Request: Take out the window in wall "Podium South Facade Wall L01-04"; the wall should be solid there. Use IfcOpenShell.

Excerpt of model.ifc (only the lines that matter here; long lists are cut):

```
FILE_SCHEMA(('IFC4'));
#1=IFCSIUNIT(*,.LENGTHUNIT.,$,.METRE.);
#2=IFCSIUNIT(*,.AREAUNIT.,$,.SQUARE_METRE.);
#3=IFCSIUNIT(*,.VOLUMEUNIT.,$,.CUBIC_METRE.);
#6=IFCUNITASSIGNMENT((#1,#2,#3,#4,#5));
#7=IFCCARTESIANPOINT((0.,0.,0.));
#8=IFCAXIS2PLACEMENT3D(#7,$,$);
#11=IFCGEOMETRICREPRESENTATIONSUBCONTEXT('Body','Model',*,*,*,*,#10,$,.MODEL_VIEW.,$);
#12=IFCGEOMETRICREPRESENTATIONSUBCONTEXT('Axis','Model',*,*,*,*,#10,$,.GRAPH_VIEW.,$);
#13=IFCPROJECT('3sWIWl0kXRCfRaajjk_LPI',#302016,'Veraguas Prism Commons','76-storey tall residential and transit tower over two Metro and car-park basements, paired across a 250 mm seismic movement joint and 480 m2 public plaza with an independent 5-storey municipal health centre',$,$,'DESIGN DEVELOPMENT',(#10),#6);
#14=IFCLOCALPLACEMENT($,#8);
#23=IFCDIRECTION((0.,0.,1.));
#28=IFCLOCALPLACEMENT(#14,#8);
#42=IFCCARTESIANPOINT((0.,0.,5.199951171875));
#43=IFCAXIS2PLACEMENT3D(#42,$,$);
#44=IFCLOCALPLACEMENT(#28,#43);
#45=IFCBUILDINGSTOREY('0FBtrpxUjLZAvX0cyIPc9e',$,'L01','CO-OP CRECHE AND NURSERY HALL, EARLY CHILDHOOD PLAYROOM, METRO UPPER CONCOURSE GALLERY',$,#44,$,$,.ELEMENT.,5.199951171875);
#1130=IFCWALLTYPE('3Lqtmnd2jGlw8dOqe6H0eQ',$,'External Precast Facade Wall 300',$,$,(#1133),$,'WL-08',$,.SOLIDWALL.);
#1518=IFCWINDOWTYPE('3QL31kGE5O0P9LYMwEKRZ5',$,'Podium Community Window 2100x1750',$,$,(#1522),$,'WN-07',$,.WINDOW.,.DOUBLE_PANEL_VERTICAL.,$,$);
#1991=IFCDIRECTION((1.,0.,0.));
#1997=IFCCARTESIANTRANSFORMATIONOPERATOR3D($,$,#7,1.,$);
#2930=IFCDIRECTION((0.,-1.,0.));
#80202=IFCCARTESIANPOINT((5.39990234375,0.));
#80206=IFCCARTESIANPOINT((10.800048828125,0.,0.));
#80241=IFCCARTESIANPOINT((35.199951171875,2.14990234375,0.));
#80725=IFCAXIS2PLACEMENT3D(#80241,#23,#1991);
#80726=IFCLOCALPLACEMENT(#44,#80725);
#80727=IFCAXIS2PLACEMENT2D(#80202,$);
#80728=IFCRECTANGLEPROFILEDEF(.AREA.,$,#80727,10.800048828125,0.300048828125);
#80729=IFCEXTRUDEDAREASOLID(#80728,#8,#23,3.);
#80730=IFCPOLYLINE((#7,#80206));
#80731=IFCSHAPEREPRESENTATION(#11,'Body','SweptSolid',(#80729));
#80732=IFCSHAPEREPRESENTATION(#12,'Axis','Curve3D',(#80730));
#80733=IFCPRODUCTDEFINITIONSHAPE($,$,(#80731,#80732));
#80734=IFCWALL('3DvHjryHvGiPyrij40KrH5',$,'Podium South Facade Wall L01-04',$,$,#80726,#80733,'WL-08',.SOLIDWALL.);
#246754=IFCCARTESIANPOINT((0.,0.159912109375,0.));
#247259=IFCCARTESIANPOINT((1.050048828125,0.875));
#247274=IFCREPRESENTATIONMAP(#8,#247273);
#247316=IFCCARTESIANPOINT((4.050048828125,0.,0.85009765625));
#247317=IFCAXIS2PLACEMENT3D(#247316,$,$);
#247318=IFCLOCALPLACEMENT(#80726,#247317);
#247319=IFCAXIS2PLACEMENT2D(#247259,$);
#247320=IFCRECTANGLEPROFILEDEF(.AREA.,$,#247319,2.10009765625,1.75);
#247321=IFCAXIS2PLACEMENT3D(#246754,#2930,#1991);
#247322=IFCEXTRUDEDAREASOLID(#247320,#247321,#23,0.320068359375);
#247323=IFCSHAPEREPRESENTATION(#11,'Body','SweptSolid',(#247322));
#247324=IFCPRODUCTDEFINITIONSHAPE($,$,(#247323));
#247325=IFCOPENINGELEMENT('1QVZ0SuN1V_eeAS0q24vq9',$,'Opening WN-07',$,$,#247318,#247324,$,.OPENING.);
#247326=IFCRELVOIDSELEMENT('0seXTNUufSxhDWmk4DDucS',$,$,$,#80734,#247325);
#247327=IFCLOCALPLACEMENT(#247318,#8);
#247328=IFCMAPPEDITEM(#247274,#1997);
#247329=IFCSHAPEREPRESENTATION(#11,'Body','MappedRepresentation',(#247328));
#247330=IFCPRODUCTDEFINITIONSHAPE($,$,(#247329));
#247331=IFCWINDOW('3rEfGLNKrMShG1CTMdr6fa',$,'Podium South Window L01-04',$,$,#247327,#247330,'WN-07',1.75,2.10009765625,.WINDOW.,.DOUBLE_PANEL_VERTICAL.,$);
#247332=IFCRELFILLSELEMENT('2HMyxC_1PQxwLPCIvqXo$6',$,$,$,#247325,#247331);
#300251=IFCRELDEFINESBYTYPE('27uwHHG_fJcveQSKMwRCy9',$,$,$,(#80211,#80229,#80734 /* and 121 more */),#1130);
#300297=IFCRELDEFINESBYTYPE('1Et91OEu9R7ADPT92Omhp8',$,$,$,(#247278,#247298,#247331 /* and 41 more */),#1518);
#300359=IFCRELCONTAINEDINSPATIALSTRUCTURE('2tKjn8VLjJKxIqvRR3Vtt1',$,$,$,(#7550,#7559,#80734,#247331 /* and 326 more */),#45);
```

```python
import ifcopenshell
import ifcopenshell.api.feature
import ifcopenshell.api.root
import ifcopenshell.geom
import ifcopenshell.util.shape

model = ifcopenshell.open("model.ifc")
settings = ifcopenshell.geom.settings()


def volume(element):
    """Net volume in cubic metres, openings subtracted."""
    shape = ifcopenshell.geom.create_shape(settings, element)
    return ifcopenshell.util.shape.get_volume(shape.geometry)


window = model.by_guid("3rEfGLNKrMShG1CTMdr6fa")
opening = window.FillsVoids[0].RelatingOpeningElement
wall = opening.VoidsElements[0].RelatingBuildingElement
before = volume(wall)

ifcopenshell.api.root.remove_product(model, product=window)
ifcopenshell.api.feature.remove_feature(model, feature=opening)

after = volume(wall)

print(f"wall volume {before:.3f} -> {after:.3f} m3")

model.write("model_rev.ifc")
```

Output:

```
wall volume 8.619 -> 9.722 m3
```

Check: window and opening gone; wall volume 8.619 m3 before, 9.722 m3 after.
